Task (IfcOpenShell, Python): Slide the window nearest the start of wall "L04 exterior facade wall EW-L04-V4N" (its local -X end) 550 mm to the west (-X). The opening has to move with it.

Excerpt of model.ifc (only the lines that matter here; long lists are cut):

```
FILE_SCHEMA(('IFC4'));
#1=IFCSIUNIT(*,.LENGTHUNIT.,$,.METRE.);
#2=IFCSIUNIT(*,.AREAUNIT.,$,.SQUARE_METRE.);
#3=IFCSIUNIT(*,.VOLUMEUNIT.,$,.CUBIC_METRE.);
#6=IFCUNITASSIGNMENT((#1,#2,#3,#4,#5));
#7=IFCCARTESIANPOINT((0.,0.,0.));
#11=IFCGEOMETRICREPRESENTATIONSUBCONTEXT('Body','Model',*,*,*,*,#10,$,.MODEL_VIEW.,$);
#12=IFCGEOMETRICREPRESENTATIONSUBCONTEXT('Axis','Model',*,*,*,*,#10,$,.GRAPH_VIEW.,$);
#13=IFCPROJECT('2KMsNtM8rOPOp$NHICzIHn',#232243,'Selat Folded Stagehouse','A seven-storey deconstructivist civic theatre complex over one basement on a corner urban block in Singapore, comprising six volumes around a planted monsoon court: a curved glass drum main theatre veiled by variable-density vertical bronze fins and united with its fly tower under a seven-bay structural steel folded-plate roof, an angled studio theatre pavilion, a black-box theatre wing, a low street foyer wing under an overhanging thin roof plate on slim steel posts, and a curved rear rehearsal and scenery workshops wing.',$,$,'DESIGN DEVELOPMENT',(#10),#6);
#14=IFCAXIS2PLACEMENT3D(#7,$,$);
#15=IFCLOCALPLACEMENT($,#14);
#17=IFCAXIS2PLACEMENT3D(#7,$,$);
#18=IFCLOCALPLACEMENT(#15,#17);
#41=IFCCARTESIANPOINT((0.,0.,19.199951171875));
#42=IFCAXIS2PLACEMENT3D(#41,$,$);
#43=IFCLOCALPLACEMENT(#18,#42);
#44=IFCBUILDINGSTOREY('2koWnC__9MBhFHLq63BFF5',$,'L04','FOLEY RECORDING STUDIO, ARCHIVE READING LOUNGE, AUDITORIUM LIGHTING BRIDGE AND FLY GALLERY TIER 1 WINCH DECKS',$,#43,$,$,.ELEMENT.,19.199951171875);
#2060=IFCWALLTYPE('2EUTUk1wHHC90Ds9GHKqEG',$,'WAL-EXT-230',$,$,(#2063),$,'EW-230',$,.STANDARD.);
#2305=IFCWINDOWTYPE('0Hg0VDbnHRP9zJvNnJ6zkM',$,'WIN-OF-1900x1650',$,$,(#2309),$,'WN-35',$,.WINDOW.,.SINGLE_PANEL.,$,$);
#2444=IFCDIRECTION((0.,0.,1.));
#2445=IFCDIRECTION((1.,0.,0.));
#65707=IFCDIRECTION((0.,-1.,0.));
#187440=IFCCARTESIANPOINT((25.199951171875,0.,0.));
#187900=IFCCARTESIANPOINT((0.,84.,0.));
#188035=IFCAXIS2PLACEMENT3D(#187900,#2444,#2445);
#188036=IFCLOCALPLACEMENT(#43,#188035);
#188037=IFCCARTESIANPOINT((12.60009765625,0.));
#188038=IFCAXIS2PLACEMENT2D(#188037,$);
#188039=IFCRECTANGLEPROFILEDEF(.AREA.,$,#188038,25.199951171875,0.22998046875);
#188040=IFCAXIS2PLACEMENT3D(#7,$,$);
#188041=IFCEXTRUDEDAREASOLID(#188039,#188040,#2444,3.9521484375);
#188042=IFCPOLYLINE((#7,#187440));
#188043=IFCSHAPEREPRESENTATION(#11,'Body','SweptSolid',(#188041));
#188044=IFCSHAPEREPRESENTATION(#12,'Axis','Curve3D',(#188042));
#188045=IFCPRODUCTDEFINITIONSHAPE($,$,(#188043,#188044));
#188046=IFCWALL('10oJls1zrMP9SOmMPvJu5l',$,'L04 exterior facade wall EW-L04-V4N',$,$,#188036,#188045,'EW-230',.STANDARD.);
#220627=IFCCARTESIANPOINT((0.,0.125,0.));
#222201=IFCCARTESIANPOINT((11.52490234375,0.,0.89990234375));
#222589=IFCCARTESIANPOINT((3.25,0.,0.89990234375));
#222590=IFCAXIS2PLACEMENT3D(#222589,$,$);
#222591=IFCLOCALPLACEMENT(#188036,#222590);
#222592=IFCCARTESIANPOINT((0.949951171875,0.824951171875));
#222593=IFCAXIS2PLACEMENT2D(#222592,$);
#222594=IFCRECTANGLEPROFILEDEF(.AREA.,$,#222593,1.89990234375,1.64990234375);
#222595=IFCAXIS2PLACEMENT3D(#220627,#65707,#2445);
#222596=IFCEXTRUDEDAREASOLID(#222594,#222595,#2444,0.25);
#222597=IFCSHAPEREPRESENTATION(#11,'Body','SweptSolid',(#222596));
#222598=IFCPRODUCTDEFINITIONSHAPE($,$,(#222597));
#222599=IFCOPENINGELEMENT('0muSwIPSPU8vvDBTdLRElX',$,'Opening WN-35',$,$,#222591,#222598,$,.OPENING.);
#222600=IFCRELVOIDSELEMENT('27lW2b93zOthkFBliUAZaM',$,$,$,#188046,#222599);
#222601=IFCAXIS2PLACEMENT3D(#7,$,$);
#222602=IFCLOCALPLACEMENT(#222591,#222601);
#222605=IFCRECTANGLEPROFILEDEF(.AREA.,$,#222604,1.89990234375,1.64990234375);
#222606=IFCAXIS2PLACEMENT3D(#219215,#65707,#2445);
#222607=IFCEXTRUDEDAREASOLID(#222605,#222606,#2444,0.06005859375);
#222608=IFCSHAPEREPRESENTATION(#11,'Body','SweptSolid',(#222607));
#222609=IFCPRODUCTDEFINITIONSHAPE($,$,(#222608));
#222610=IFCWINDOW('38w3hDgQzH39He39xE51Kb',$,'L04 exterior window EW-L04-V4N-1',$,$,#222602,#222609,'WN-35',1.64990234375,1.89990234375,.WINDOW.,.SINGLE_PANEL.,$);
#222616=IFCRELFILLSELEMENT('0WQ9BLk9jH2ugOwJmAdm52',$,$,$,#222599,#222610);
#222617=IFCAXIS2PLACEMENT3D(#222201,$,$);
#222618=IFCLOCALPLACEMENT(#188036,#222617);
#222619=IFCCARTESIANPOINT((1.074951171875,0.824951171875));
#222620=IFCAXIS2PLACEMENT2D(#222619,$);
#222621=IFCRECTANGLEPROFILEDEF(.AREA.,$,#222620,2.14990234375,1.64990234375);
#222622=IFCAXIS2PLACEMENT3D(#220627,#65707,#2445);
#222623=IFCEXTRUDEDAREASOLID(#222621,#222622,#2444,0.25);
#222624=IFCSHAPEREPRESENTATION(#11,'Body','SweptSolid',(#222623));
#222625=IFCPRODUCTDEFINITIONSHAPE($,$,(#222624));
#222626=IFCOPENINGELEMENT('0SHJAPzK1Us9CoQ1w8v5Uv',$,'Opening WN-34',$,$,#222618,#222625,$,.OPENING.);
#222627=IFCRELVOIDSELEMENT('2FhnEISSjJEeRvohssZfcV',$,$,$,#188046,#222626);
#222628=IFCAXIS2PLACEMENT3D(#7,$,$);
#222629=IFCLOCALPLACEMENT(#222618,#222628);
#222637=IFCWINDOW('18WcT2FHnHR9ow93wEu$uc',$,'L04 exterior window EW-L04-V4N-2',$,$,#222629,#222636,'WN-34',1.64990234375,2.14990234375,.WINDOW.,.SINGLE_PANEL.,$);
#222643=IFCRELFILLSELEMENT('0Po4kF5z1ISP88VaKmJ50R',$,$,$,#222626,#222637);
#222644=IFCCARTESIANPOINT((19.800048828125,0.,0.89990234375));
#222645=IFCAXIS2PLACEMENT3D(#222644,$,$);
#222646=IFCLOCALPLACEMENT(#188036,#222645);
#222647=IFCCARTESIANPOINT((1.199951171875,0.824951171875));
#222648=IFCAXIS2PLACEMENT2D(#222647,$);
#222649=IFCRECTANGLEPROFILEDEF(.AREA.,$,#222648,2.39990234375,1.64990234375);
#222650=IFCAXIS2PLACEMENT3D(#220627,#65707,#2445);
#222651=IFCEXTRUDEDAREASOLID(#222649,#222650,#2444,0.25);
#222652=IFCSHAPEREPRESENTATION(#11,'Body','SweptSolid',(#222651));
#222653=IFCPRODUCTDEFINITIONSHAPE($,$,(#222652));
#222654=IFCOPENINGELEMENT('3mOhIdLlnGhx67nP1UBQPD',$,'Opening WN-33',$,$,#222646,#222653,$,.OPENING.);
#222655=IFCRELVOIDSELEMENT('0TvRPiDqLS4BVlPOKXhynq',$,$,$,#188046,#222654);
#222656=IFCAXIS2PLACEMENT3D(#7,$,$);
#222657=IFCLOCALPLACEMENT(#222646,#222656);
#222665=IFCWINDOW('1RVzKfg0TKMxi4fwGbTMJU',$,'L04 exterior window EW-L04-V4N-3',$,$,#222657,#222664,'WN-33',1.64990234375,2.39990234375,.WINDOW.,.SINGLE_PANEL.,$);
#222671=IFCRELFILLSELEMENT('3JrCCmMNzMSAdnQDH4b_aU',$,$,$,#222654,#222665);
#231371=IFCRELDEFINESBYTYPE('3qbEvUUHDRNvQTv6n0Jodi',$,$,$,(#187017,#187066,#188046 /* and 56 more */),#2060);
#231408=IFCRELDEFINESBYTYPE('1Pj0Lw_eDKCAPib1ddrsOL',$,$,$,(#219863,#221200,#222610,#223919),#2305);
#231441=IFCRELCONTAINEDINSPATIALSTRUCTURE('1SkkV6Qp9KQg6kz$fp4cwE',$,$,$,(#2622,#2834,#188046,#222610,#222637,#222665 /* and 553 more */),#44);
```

```python
import ifcopenshell
import ifcopenshell.api.geometry
import ifcopenshell.util.placement

model = ifcopenshell.open("model.ifc")

window = model.by_guid("38w3hDgQzH39He39xE51Kb")
opening = window.FillsVoids[0].RelatingOpeningElement
wall = opening.VoidsElements[0].RelatingBuildingElement

wall_matrix = ifcopenshell.util.placement.get_local_placement(wall.ObjectPlacement)
shift = wall_matrix[:3, 0] * -0.55
before = ifcopenshell.util.placement.get_local_placement(window.ObjectPlacement)[:3, 3].copy()

# The window is placed relative to its opening, so it follows when the opening moves.
matrix = ifcopenshell.util.placement.get_local_placement(opening.ObjectPlacement)
matrix[:3, 3] += shift
ifcopenshell.api.geometry.edit_object_placement(
    model, product=opening, matrix=matrix, is_si=False, should_transform_children=True
)

after = ifcopenshell.util.placement.get_local_placement(window.ObjectPlacement)[:3, 3]
print("window moved by", (after - before).round(3) + 0.0)

model.write("model-out.ifc")
```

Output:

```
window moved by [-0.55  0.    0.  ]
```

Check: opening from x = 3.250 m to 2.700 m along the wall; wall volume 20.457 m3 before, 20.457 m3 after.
